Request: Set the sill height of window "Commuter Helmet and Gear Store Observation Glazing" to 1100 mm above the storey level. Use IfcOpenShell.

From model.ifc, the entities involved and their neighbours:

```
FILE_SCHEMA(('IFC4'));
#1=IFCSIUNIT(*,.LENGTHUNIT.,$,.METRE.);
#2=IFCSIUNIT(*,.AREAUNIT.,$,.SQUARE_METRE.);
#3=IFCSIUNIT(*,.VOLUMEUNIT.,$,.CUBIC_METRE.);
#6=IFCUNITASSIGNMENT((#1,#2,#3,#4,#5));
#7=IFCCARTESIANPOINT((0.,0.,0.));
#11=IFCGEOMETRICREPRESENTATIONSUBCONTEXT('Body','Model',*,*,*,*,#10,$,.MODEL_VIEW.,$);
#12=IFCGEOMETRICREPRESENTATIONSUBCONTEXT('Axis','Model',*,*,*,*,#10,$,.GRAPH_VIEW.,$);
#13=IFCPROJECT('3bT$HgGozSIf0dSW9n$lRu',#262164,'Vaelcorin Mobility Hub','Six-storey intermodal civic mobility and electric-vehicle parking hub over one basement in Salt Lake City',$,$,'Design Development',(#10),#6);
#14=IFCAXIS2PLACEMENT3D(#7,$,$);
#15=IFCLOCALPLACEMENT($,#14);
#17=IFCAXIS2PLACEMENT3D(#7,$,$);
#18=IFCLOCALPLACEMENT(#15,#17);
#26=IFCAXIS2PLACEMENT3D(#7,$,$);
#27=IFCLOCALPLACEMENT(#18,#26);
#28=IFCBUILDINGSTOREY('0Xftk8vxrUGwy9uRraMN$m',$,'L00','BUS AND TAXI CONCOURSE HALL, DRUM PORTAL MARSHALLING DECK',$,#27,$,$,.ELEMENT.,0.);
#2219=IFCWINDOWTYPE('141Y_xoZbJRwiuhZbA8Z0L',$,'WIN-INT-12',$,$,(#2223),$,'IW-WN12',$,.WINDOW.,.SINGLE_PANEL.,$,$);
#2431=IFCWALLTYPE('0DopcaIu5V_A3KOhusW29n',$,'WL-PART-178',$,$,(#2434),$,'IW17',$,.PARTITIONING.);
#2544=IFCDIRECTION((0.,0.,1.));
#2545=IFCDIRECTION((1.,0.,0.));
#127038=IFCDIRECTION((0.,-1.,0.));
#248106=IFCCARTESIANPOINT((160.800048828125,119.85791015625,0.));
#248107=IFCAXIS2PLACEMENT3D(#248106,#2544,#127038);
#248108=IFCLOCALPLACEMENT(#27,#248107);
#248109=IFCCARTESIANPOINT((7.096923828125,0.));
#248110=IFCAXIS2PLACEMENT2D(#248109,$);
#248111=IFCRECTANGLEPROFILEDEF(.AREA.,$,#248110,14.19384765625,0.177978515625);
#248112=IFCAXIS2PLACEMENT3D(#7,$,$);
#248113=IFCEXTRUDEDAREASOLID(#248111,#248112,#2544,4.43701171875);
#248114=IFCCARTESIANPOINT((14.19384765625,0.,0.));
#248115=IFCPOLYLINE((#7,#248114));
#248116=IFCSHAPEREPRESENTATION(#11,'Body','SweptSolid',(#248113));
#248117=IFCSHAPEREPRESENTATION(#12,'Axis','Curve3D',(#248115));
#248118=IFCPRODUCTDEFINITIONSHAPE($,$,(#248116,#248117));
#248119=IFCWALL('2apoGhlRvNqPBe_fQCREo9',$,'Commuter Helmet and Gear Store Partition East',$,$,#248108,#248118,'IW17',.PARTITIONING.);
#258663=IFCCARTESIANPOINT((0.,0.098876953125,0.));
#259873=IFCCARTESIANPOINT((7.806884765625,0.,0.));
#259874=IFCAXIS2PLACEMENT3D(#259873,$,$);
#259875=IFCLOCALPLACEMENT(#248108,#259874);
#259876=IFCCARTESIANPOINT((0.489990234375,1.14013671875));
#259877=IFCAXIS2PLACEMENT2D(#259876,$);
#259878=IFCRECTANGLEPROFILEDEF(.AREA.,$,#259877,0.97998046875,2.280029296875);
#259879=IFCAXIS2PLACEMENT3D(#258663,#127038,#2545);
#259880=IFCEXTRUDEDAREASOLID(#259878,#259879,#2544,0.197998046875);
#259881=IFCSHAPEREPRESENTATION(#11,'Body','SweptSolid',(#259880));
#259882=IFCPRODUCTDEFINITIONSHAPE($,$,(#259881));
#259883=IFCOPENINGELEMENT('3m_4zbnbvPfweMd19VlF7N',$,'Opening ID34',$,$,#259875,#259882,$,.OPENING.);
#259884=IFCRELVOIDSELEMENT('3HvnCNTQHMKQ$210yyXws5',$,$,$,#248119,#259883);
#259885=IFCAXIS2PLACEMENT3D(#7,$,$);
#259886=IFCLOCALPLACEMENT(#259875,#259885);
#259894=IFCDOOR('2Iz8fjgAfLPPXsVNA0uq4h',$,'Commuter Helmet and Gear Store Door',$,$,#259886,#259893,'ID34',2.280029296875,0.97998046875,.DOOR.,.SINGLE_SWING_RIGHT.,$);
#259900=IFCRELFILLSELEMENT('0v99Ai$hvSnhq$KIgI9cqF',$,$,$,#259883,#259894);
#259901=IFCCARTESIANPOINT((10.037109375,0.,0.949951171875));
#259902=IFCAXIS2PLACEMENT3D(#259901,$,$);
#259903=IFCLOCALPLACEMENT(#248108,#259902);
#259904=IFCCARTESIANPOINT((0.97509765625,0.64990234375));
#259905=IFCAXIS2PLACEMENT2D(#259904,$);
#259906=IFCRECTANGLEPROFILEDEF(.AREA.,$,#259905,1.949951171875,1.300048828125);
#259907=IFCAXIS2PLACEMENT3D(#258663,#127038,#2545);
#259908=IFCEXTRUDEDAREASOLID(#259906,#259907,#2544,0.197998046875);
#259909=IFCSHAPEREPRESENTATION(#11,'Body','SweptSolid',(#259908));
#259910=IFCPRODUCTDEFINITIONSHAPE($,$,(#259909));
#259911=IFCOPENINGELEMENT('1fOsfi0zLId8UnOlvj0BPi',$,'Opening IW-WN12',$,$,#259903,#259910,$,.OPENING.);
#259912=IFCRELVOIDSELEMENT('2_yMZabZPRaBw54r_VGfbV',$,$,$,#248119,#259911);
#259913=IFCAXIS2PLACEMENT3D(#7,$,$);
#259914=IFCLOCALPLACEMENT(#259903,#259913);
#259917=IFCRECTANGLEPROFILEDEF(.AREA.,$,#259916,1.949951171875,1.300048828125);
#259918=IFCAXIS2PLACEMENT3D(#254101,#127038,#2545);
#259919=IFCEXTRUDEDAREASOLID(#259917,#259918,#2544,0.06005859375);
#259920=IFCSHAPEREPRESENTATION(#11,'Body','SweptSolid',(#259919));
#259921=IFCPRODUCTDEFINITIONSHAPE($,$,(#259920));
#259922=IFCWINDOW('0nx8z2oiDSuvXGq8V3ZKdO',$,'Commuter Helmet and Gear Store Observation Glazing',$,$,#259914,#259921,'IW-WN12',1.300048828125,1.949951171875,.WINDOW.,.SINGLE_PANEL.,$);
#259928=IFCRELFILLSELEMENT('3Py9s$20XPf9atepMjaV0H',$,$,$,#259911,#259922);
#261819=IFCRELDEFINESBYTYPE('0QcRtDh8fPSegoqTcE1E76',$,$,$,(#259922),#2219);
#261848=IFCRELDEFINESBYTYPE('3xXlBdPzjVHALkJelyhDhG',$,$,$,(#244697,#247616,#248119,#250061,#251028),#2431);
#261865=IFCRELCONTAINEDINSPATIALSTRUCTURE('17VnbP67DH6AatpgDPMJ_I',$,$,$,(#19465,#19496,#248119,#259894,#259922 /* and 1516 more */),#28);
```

```python
import numpy as np
import ifcopenshell
import ifcopenshell.api.geometry
import ifcopenshell.geom
import ifcopenshell.util.element
import ifcopenshell.util.placement
import ifcopenshell.util.shape
import ifcopenshell.util.unit

model = ifcopenshell.open("model.ifc")
unit_scale = ifcopenshell.util.unit.calculate_unit_scale(model)

window = model.by_guid("0nx8z2oiDSuvXGq8V3ZKdO")
opening = window.FillsVoids[0].RelatingOpeningElement
storey = ifcopenshell.util.element.get_container(window, ifc_class="IfcBuildingStorey")
level = ifcopenshell.util.placement.get_local_placement(storey.ObjectPlacement)[2, 3]

# The opening's origin need not be at the sill, so measure its lowest point.
shape = ifcopenshell.geom.create_shape(ifcopenshell.geom.settings(), opening)
bottom = ifcopenshell.util.shape.get_shape_bottom_elevation(shape, shape.geometry) / unit_scale
dz = level + 1.1 / unit_scale - bottom

shift = np.array([0.0, 0.0, dz])
# The window is placed relative to its opening, so it follows when the opening moves.
matrix = ifcopenshell.util.placement.get_local_placement(opening.ObjectPlacement)
matrix[:3, 3] += shift
ifcopenshell.api.geometry.edit_object_placement(
    model, product=opening, matrix=matrix, is_si=False, should_transform_children=True
)

print(f"moved by {dz * unit_scale:+.3f} m")

model.write("model_edited.ifc")
```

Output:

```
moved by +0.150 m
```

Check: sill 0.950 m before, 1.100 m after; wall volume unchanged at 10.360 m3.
